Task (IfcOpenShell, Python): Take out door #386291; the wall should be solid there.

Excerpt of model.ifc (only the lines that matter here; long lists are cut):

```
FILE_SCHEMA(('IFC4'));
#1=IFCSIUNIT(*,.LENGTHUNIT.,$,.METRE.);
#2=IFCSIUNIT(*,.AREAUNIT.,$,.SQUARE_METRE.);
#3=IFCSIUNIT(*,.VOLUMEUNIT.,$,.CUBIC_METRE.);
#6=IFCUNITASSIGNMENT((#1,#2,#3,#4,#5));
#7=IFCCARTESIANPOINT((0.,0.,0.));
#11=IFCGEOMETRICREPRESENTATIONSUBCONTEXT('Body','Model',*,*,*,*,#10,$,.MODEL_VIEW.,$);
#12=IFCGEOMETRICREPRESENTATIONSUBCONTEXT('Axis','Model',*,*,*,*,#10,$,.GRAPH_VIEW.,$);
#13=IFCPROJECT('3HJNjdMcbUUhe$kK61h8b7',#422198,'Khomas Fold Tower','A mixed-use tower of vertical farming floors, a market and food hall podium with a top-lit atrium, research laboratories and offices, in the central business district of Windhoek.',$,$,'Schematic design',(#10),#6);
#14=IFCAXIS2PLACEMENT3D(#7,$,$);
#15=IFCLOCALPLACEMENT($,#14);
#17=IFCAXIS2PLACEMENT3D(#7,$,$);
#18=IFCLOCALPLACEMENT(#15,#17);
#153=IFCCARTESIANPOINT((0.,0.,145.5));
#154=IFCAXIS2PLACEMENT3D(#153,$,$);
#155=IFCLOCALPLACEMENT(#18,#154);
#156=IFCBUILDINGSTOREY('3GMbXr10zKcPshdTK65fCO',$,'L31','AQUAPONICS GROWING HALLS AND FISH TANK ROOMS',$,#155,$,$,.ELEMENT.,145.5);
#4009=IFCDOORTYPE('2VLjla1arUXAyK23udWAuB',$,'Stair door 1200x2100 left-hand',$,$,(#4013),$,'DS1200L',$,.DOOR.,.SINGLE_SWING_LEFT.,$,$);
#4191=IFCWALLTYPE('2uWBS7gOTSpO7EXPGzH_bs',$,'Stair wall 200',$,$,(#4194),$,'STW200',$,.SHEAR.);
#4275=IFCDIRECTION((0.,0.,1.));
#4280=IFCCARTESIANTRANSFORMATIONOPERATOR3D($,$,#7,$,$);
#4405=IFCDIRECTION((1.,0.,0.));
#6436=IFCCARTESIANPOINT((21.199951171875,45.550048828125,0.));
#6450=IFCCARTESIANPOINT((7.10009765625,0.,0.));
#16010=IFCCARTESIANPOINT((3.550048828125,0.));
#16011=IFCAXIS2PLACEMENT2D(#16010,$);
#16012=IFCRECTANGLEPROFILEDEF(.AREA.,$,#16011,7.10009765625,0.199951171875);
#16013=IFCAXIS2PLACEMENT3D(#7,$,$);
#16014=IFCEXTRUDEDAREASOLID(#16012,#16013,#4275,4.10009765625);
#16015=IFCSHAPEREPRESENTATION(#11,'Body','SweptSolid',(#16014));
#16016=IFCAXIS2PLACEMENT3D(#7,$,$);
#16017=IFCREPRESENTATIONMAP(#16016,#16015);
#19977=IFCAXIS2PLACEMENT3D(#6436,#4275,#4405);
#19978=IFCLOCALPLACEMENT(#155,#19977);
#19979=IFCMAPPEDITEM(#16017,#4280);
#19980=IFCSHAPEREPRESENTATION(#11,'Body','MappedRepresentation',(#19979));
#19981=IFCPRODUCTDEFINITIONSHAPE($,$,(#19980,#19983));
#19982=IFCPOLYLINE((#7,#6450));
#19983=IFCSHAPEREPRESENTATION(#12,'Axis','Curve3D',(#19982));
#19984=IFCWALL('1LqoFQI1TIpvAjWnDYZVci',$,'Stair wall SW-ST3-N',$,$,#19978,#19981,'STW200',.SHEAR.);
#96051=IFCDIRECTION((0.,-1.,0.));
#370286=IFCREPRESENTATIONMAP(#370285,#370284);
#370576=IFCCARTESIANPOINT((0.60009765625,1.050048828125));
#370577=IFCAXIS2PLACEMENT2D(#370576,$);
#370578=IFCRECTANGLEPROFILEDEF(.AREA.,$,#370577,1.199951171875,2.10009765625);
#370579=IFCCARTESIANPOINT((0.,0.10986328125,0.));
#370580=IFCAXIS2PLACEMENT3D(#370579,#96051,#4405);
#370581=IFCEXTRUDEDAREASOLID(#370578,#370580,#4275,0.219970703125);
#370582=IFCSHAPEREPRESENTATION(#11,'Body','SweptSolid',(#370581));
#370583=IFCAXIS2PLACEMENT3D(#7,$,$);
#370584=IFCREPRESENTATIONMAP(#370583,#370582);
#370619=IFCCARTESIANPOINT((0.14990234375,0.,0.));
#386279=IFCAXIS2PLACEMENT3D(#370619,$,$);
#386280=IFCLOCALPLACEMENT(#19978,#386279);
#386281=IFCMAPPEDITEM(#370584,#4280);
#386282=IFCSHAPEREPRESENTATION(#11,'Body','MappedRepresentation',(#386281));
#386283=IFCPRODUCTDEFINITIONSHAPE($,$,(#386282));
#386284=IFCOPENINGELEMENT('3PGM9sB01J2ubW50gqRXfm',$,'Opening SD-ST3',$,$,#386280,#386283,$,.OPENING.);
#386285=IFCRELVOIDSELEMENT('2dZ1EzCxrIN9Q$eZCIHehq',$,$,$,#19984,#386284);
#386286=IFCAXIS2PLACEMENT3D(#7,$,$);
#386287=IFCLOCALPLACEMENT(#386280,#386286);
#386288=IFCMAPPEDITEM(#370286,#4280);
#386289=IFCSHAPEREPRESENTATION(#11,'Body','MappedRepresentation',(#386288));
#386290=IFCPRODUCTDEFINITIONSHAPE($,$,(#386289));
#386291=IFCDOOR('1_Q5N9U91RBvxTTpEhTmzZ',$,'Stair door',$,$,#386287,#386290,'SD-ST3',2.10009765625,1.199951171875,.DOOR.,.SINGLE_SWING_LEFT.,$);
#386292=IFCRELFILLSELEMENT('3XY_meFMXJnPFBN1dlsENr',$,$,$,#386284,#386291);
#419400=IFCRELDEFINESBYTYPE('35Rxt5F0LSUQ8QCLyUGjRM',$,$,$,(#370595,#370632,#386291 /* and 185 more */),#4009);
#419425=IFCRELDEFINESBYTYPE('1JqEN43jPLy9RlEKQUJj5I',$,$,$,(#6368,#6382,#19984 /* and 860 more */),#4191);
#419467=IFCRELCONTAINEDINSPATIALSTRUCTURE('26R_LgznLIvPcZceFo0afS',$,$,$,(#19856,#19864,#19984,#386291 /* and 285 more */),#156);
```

```python
import ifcopenshell
import ifcopenshell.api.feature
import ifcopenshell.api.root
import ifcopenshell.geom
import ifcopenshell.util.shape

model = ifcopenshell.open("model.ifc")
settings = ifcopenshell.geom.settings()


def volume(element):
    """Net volume in cubic metres, openings subtracted."""
    shape = ifcopenshell.geom.create_shape(settings, element)
    return ifcopenshell.util.shape.get_volume(shape.geometry)


door = model.by_guid("1_Q5N9U91RBvxTTpEhTmzZ")
opening = door.FillsVoids[0].RelatingOpeningElement
wall = opening.VoidsElements[0].RelatingBuildingElement
before = volume(wall)

ifcopenshell.api.root.remove_product(model, product=door)
ifcopenshell.api.feature.remove_feature(model, feature=opening)

after = volume(wall)

print(f"wall volume {before:.3f} -> {after:.3f} m3")

model.write("model_rev.ifc")
```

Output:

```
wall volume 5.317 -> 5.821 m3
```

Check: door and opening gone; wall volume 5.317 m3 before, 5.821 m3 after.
